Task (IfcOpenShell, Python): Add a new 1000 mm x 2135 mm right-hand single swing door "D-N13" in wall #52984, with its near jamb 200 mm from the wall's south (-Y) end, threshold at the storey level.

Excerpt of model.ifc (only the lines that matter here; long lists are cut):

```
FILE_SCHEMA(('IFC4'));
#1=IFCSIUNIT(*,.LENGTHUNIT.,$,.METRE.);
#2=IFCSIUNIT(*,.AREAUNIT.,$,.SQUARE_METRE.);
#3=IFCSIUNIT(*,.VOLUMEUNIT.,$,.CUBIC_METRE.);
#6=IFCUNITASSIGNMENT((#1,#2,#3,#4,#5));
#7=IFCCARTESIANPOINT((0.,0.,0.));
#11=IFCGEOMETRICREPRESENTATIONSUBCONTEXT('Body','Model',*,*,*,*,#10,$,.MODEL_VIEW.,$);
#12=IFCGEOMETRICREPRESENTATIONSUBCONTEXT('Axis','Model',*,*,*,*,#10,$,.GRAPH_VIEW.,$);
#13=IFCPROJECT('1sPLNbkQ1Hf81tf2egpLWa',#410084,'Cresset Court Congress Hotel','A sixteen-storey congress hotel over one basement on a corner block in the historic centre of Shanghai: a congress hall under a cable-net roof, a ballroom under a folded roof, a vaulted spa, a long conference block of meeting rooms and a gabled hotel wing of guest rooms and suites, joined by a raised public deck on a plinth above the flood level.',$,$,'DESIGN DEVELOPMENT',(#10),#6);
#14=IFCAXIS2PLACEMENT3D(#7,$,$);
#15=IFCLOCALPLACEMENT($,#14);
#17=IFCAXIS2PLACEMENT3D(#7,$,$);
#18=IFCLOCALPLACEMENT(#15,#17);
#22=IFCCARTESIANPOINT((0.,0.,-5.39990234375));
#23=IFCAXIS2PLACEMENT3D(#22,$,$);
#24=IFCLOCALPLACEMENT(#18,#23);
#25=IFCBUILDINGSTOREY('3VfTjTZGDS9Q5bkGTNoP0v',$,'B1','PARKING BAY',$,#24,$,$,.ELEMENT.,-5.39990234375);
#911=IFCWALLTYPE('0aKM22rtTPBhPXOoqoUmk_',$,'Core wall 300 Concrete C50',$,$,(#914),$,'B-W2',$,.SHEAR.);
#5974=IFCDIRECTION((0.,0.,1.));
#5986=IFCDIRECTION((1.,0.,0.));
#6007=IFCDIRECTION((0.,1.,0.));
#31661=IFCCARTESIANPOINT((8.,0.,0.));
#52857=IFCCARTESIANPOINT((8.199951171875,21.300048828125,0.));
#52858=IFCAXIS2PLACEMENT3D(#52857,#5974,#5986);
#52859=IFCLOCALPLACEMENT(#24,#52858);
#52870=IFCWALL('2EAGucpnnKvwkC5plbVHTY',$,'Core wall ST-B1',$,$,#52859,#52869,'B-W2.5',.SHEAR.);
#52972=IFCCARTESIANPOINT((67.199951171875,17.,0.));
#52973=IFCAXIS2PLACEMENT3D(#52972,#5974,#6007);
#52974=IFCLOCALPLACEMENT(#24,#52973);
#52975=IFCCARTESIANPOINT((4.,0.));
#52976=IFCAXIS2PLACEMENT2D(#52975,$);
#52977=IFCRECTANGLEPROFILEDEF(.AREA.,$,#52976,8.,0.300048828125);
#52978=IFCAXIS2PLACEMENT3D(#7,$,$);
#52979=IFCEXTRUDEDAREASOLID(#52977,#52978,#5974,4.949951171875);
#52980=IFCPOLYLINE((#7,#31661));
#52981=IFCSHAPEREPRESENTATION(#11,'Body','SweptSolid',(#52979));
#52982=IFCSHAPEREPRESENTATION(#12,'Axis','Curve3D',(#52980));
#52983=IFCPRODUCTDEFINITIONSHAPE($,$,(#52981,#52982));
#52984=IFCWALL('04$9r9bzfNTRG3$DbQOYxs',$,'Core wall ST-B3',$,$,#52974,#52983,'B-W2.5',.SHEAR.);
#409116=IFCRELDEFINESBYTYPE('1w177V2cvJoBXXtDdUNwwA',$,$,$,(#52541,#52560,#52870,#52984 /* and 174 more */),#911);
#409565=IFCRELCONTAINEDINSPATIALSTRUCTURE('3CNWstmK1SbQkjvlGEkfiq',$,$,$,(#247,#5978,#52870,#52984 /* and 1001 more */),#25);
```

```python
import numpy as np
import ifcopenshell
import ifcopenshell.api.feature
import ifcopenshell.api.geometry
import ifcopenshell.api.root
import ifcopenshell.api.spatial
import ifcopenshell.geom
import ifcopenshell.util.element
import ifcopenshell.util.placement
import ifcopenshell.util.representation
import ifcopenshell.util.shape
import ifcopenshell.util.unit

model = ifcopenshell.open("model.ifc")
unit_scale = ifcopenshell.util.unit.calculate_unit_scale(model)
settings = ifcopenshell.geom.settings()


def volume(element):
    """Net volume in cubic metres, openings subtracted."""
    shape = ifcopenshell.geom.create_shape(settings, element)
    return ifcopenshell.util.shape.get_volume(shape.geometry)


wall = model.by_guid("04$9r9bzfNTRG3$DbQOYxs")
storey = ifcopenshell.util.element.get_container(wall, ifc_class="IfcBuildingStorey")
context = ifcopenshell.util.representation.get_context(model, "Model", "Body", "MODEL_VIEW")
before = volume(wall)

width, height, from_end, sill = 1, 2.135, 0.2, 0.0  # metres

# The wall runs along its own X axis, and the end named is its -X end.
wall_shape = ifcopenshell.geom.create_shape(settings, wall)
x, y, z = ifcopenshell.util.shape.get_vertices(wall_shape.geometry).T
start = x.min() + from_end
face, thickness = float(y.min()), float(y.max() - y.min())
wall_matrix = ifcopenshell.util.placement.get_local_placement(wall.ObjectPlacement)
level = ifcopenshell.util.placement.get_local_placement(storey.ObjectPlacement)[2, 3]


def in_wall(x, y):
    """Placement at x, y metres in the wall's axes, at sill height."""
    matrix = wall_matrix.copy()
    matrix[:, 3] = wall_matrix @ np.array([x / unit_scale, y / unit_scale, 0.0, 1.0])
    matrix[2, 3] = level + sill / unit_scale
    return matrix


# Opening: a box that overshoots both wall faces by 50 mm.
opening = ifcopenshell.api.root.create_entity(model, ifc_class="IfcOpeningElement", predefined_type="OPENING")
box = ifcopenshell.api.geometry.add_wall_representation(
    model, context=context, length=width, height=height, thickness=thickness + 0.1
)
ifcopenshell.api.geometry.assign_representation(model, product=opening, representation=box)
ifcopenshell.api.geometry.edit_object_placement(model, product=opening, matrix=in_wall(start, face - 0.05), is_si=False)
ifcopenshell.api.feature.add_feature(model, feature=opening, element=wall)

door = ifcopenshell.api.root.create_entity(model, ifc_class="IfcDoor", name="D-N13", predefined_type="DOOR")
door.OverallWidth, door.OverallHeight = width / unit_scale, height / unit_scale
door.OperationType = "SINGLE_SWING_RIGHT"
body = ifcopenshell.api.geometry.add_door_representation(
    model,
    context=context,
    overall_width=door.OverallWidth,
    overall_height=door.OverallHeight,
    operation_type="SINGLE_SWING_RIGHT",
    lining_properties={"LiningDepth": thickness / unit_scale, "ThresholdDepth": thickness / unit_scale},
)
ifcopenshell.api.geometry.assign_representation(model, product=door, representation=body)
ifcopenshell.api.spatial.assign_container(model, products=[door], relating_structure=storey)
ifcopenshell.api.feature.add_filling(model, opening=opening, element=door)

# The lining spans the wall, so the door starts at the wall face.
ifcopenshell.api.geometry.edit_object_placement(model, product=door, matrix=in_wall(start, face), is_si=False)

after = volume(wall)

print(f"wall volume {before:.3f} -> {after:.3f} m3")

model.write("model_rev.ifc")
```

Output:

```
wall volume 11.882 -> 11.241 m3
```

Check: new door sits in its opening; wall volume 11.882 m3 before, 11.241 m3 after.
